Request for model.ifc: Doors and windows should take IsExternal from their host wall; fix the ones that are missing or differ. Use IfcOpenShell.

First a look at what the model holds.

```python
import ifcopenshell
import ifcopenshell.util.element

model = ifcopenshell.open("model.ifc")
print(model.schema)
seen = {}
for e in model.by_type("IfcDoor") + model.by_type("IfcWindow"):
    if not e.FillsVoids:
        continue
    host = e.FillsVoids[0].RelatingOpeningElement.VoidsElements[0].RelatingBuildingElement
    own = ifcopenshell.util.element.get_pset(e, f"Pset_{e.is_a()[3:].removesuffix('StandardCase')}Common", "IsExternal")
    wall = ifcopenshell.util.element.get_pset(host, "Pset_WallCommon", "IsExternal")
    seen[e.is_a(), own, wall] = seen.get((e.is_a(), own, wall), 0) + 1
for (cls, own, wall), count in sorted(seen.items(), key=str):
    print(count, cls, "IsExternal:", own, "| host wall:", wall)
```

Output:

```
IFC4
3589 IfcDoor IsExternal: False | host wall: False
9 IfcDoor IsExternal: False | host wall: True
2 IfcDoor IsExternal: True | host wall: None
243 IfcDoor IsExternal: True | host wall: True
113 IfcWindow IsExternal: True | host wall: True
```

```python
import ifcopenshell
import ifcopenshell.api.pset
import ifcopenshell.util.element

model = ifcopenshell.open("model.ifc")

count = 0
for ifc_class, pset_name in (("IfcDoor", "Pset_DoorCommon"), ("IfcWindow", "Pset_WindowCommon")):
    for e in model.by_type(ifc_class):
        if not e.FillsVoids:
            continue
        host = e.FillsVoids[0].RelatingOpeningElement.VoidsElements[0].RelatingBuildingElement
        external = ifcopenshell.util.element.get_pset(host, "Pset_WallCommon", "IsExternal")
        if external is None or ifcopenshell.util.element.get_pset(e, pset_name, "IsExternal") == external:
            continue
        found = ifcopenshell.util.element.get_pset(e, pset_name, should_inherit=False)
        if found:
            pset = model.by_id(found["id"])
            if len(ifcopenshell.util.element.get_elements_by_pset(pset)) > 1:
                pset = ifcopenshell.api.pset.unshare_pset(model, products=[e], pset=pset)[0]
        else:
            pset = ifcopenshell.api.pset.add_pset(model, product=e, name=pset_name)
        ifcopenshell.api.pset.edit_pset(model, pset=pset, properties={"IsExternal": external})
        count += 1

print(count, "updated")

model.write("model_rev.ifc")
```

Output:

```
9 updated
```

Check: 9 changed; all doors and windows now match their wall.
